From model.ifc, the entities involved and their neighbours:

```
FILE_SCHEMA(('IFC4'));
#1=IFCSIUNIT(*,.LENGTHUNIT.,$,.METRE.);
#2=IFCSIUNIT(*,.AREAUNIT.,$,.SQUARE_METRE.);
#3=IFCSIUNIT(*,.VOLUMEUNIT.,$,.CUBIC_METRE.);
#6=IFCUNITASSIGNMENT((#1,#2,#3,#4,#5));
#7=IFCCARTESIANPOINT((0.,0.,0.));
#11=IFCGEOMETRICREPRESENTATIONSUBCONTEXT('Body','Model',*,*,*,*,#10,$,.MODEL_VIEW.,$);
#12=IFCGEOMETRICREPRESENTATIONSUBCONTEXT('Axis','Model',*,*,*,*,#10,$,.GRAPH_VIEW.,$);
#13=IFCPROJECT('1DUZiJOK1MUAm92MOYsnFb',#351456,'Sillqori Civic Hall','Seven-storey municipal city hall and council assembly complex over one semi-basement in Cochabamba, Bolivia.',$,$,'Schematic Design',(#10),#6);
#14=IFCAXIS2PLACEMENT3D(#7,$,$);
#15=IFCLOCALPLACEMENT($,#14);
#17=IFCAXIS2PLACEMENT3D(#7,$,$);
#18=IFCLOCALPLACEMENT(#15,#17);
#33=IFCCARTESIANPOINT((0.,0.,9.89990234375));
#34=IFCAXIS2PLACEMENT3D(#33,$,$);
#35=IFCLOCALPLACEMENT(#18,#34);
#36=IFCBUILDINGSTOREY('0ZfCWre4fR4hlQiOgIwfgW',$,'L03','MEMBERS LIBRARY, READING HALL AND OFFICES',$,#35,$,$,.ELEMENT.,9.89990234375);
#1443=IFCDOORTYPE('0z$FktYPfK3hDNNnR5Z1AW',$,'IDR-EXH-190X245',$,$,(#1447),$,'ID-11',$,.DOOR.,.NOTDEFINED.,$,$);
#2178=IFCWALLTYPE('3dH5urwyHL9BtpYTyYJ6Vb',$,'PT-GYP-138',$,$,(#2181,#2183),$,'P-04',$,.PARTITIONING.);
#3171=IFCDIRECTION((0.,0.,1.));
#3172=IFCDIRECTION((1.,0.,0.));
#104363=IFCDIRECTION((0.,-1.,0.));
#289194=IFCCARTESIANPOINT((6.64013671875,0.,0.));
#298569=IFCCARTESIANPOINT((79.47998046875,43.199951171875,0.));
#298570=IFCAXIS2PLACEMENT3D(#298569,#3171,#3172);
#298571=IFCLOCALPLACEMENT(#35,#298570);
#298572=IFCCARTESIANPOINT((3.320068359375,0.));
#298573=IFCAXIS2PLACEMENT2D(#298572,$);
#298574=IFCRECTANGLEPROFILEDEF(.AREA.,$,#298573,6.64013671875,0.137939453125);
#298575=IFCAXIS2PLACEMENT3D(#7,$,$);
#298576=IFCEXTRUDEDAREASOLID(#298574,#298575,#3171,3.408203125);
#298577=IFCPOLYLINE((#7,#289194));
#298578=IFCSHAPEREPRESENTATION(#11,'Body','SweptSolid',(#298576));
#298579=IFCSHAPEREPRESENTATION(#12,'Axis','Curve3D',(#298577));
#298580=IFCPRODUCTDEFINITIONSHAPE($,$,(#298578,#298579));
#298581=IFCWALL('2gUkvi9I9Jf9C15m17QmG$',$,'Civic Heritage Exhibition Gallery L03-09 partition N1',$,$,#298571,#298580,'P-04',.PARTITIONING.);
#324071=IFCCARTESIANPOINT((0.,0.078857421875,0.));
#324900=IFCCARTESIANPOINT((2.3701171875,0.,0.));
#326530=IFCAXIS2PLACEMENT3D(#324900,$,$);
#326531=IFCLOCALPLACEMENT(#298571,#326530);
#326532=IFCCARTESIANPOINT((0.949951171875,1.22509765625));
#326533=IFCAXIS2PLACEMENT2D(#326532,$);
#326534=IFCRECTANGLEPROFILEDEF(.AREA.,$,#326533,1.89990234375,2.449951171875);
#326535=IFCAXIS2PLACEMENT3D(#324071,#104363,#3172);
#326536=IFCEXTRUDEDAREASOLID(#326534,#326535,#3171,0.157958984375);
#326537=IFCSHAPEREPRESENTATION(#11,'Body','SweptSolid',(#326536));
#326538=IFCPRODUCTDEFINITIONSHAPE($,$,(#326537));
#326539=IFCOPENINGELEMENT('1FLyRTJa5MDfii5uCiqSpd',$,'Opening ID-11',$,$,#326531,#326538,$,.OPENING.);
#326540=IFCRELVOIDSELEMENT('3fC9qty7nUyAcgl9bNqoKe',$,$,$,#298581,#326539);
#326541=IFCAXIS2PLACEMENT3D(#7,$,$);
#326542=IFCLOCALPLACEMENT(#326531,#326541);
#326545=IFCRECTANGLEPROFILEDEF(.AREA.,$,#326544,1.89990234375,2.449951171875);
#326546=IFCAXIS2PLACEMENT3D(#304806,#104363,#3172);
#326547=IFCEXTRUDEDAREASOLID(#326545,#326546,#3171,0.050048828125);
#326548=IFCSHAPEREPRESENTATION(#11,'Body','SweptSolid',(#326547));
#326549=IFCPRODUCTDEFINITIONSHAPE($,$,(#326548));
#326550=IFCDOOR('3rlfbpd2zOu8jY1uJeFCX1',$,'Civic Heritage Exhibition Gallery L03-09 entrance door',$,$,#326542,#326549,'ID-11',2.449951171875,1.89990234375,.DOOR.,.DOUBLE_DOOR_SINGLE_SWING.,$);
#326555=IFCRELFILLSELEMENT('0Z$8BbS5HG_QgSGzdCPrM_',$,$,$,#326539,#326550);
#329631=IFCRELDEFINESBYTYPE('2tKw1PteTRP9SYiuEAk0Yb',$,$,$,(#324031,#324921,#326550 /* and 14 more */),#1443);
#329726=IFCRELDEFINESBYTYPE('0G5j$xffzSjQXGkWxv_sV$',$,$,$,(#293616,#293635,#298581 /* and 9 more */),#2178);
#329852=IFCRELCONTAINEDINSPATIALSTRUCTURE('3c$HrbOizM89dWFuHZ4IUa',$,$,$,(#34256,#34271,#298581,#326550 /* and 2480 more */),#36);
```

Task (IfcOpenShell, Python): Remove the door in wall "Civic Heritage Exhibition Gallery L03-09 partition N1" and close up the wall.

```python
import ifcopenshell
import ifcopenshell.api.feature
import ifcopenshell.api.root
import ifcopenshell.geom
import ifcopenshell.util.shape

model = ifcopenshell.open("model.ifc")
settings = ifcopenshell.geom.settings()


def volume(element):
    """Net volume in cubic metres, openings subtracted."""
    shape = ifcopenshell.geom.create_shape(settings, element)
    return ifcopenshell.util.shape.get_volume(shape.geometry)


door = model.by_guid("3rlfbpd2zOu8jY1uJeFCX1")
opening = door.FillsVoids[0].RelatingOpeningElement
wall = opening.VoidsElements[0].RelatingBuildingElement
before = volume(wall)

ifcopenshell.api.root.remove_product(model, product=door)
ifcopenshell.api.feature.remove_feature(model, feature=opening)

after = volume(wall)

print(f"wall volume {before:.3f} -> {after:.3f} m3")

model.write("model_updated.ifc")
```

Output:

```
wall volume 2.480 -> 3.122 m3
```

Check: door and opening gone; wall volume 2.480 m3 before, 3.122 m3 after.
